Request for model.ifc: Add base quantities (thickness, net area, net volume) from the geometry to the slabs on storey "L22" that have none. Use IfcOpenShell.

First a look at what the model holds.

```python
import ifcopenshell
import ifcopenshell.util.element
import ifcopenshell.util.unit

model = ifcopenshell.open("model.ifc")
print(model.schema)
for unit_type in ("LENGTHUNIT", "AREAUNIT", "VOLUMEUNIT"):
    print(unit_type, ifcopenshell.util.unit.calculate_unit_scale(model, unit_type))
storey = next(s for s in model.by_type("IfcBuildingStorey") if s.Name == "L22")
slabs = [e for e in ifcopenshell.util.element.get_decomposition(storey) if e.is_a("IfcSlab")]
for e in sorted(slabs, key=lambda e: e.id()):
    print(e.id(), e.is_a(), e.Name, list(ifcopenshell.util.element.get_psets(e, qtos_only=True)), sep=" | ")
```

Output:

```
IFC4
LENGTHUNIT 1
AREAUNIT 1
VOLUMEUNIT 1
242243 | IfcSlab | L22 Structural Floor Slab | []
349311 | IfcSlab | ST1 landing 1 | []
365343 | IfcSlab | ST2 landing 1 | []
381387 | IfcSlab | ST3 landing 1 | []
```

```python
import ifcopenshell
import ifcopenshell.api.pset
import ifcopenshell.geom
import ifcopenshell.util.element
import ifcopenshell.util.shape
import ifcopenshell.util.unit

model = ifcopenshell.open("model.ifc")
unit_scale = ifcopenshell.util.unit.calculate_unit_scale(model)
area_scale = ifcopenshell.util.unit.calculate_unit_scale(model, "AREAUNIT")
volume_scale = ifcopenshell.util.unit.calculate_unit_scale(model, "VOLUMEUNIT")
settings = ifcopenshell.geom.settings()

storey = next(s for s in model.by_type("IfcBuildingStorey") if s.Name == "L22")
slabs = [e for e in ifcopenshell.util.element.get_decomposition(storey) if e.is_a("IfcSlab")]

for e in sorted(slabs, key=lambda e: e.id()):
    if ifcopenshell.util.element.get_psets(e, qtos_only=True, should_inherit=False):
        continue
    # Geometry comes back in metres, in the element's own axes.
    shape = ifcopenshell.geom.create_shape(settings, e)
    values = {
        "Width": ifcopenshell.util.shape.get_z(shape.geometry) / unit_scale,
        "NetArea": ifcopenshell.util.shape.get_footprint_area(shape.geometry) / area_scale,
        "NetVolume": ifcopenshell.util.shape.get_volume(shape.geometry) / volume_scale,
    }
    qto = ifcopenshell.api.pset.add_qto(model, product=e, name="Qto_SlabBaseQuantities")
    ifcopenshell.api.pset.edit_qto(model, qto=qto, properties=values)
    print(e.id(), {k: round(v, 3) for k, v in values.items()})

model.write("model_v2.ifc")
```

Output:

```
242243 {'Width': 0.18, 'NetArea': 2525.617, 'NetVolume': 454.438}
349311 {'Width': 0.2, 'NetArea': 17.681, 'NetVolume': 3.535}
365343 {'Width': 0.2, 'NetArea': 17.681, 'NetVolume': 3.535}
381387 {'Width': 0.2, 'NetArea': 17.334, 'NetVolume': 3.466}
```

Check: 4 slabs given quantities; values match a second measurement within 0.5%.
